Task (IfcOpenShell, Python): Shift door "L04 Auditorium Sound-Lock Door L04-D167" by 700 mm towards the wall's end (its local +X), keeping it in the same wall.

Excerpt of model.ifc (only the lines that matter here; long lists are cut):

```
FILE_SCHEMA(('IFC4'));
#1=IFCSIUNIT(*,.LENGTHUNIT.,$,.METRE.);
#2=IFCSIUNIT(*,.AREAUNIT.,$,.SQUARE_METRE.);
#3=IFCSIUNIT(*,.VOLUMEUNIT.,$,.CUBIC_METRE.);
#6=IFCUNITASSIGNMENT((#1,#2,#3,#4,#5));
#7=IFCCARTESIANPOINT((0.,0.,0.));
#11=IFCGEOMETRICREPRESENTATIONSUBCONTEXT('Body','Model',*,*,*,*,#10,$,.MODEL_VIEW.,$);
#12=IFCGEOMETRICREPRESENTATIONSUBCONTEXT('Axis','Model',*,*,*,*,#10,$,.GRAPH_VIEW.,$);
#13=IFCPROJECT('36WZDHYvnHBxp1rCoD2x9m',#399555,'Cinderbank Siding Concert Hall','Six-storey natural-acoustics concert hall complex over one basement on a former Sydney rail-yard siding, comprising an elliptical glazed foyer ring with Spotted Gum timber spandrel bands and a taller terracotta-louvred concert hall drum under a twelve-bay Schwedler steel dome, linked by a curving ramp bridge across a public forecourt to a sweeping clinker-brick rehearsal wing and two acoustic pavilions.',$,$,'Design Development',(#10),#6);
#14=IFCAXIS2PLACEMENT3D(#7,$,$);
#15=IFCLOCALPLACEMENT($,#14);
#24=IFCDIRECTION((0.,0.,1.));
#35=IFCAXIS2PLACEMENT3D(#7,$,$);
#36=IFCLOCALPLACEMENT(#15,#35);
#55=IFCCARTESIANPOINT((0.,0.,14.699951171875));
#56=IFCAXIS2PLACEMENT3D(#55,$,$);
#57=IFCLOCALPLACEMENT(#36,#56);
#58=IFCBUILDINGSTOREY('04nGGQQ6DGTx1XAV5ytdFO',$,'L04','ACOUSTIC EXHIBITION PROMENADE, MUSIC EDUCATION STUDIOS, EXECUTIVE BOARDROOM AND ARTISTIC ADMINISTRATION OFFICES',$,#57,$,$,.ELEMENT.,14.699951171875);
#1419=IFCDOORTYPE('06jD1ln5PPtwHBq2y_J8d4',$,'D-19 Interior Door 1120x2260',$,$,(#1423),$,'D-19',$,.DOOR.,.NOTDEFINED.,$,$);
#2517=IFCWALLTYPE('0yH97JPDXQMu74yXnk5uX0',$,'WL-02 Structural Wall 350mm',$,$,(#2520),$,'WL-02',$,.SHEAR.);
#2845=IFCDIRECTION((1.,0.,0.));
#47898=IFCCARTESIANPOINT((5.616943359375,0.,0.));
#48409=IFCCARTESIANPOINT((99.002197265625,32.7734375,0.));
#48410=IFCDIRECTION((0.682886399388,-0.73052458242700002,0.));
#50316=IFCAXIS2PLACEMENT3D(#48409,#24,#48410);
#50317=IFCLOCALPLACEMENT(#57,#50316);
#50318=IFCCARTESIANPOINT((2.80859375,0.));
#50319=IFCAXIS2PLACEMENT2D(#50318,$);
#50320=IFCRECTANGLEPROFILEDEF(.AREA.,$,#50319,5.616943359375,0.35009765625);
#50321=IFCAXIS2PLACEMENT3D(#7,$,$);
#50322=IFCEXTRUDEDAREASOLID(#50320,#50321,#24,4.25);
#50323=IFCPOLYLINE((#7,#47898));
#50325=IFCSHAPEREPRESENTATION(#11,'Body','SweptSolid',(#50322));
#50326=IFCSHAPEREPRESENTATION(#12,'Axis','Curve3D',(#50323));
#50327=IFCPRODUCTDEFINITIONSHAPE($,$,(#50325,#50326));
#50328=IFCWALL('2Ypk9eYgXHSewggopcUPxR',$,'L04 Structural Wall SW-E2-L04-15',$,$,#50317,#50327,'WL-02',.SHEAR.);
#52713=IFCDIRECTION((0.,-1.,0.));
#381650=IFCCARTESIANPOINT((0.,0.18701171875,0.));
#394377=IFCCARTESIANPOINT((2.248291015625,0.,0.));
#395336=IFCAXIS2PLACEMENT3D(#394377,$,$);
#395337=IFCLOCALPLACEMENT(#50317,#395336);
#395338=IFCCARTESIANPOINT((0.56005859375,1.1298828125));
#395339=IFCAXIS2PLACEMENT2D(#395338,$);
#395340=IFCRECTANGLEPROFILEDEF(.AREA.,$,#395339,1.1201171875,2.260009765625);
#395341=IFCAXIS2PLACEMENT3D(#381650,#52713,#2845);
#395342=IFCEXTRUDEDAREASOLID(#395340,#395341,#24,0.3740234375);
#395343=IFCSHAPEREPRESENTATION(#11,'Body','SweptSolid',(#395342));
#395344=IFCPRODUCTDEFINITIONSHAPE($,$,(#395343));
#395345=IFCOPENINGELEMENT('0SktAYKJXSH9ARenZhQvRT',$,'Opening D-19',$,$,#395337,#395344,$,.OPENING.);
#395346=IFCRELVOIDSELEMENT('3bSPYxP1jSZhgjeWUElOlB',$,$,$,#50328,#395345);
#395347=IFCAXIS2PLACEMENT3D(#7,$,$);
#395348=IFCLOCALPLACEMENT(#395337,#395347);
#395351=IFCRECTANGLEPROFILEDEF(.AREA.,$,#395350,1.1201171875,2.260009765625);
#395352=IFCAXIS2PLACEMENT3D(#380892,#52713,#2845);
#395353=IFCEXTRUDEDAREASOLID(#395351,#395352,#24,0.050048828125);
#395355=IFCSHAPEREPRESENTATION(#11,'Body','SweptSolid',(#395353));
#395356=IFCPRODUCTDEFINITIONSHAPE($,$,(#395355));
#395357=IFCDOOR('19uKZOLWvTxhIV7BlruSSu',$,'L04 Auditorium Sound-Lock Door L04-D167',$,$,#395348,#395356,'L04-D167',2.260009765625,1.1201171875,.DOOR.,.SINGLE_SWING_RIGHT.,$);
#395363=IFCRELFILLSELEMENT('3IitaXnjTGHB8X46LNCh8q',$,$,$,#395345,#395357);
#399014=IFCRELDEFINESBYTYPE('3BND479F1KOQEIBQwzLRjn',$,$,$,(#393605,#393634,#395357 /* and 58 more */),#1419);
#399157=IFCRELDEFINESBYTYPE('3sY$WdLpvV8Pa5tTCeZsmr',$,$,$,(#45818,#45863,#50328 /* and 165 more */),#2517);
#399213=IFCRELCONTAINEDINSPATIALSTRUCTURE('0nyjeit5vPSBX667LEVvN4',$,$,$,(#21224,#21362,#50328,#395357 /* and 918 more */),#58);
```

```python
import ifcopenshell
import ifcopenshell.api.geometry
import ifcopenshell.util.placement
import ifcopenshell.util.unit

model = ifcopenshell.open("model.ifc")
unit_scale = ifcopenshell.util.unit.calculate_unit_scale(model)

door = model.by_guid("19uKZOLWvTxhIV7BlruSSu")
opening = door.FillsVoids[0].RelatingOpeningElement
wall = opening.VoidsElements[0].RelatingBuildingElement

wall_matrix = ifcopenshell.util.placement.get_local_placement(wall.ObjectPlacement)
shift = wall_matrix[:3, 0] * 0.7 / unit_scale
before = ifcopenshell.util.placement.get_local_placement(door.ObjectPlacement)[:3, 3].copy()

# The door is placed relative to its opening, so it follows when the opening moves.
matrix = ifcopenshell.util.placement.get_local_placement(opening.ObjectPlacement)
matrix[:3, 3] += shift
ifcopenshell.api.geometry.edit_object_placement(
    model, product=opening, matrix=matrix, is_si=False, should_transform_children=True
)

after = ifcopenshell.util.placement.get_local_placement(door.ObjectPlacement)[:3, 3]
print("door moved by", (after - before).round(3) + 0.0)

model.write("model_v2.ifc")
```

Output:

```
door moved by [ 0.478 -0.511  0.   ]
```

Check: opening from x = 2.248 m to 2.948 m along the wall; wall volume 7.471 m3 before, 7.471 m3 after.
